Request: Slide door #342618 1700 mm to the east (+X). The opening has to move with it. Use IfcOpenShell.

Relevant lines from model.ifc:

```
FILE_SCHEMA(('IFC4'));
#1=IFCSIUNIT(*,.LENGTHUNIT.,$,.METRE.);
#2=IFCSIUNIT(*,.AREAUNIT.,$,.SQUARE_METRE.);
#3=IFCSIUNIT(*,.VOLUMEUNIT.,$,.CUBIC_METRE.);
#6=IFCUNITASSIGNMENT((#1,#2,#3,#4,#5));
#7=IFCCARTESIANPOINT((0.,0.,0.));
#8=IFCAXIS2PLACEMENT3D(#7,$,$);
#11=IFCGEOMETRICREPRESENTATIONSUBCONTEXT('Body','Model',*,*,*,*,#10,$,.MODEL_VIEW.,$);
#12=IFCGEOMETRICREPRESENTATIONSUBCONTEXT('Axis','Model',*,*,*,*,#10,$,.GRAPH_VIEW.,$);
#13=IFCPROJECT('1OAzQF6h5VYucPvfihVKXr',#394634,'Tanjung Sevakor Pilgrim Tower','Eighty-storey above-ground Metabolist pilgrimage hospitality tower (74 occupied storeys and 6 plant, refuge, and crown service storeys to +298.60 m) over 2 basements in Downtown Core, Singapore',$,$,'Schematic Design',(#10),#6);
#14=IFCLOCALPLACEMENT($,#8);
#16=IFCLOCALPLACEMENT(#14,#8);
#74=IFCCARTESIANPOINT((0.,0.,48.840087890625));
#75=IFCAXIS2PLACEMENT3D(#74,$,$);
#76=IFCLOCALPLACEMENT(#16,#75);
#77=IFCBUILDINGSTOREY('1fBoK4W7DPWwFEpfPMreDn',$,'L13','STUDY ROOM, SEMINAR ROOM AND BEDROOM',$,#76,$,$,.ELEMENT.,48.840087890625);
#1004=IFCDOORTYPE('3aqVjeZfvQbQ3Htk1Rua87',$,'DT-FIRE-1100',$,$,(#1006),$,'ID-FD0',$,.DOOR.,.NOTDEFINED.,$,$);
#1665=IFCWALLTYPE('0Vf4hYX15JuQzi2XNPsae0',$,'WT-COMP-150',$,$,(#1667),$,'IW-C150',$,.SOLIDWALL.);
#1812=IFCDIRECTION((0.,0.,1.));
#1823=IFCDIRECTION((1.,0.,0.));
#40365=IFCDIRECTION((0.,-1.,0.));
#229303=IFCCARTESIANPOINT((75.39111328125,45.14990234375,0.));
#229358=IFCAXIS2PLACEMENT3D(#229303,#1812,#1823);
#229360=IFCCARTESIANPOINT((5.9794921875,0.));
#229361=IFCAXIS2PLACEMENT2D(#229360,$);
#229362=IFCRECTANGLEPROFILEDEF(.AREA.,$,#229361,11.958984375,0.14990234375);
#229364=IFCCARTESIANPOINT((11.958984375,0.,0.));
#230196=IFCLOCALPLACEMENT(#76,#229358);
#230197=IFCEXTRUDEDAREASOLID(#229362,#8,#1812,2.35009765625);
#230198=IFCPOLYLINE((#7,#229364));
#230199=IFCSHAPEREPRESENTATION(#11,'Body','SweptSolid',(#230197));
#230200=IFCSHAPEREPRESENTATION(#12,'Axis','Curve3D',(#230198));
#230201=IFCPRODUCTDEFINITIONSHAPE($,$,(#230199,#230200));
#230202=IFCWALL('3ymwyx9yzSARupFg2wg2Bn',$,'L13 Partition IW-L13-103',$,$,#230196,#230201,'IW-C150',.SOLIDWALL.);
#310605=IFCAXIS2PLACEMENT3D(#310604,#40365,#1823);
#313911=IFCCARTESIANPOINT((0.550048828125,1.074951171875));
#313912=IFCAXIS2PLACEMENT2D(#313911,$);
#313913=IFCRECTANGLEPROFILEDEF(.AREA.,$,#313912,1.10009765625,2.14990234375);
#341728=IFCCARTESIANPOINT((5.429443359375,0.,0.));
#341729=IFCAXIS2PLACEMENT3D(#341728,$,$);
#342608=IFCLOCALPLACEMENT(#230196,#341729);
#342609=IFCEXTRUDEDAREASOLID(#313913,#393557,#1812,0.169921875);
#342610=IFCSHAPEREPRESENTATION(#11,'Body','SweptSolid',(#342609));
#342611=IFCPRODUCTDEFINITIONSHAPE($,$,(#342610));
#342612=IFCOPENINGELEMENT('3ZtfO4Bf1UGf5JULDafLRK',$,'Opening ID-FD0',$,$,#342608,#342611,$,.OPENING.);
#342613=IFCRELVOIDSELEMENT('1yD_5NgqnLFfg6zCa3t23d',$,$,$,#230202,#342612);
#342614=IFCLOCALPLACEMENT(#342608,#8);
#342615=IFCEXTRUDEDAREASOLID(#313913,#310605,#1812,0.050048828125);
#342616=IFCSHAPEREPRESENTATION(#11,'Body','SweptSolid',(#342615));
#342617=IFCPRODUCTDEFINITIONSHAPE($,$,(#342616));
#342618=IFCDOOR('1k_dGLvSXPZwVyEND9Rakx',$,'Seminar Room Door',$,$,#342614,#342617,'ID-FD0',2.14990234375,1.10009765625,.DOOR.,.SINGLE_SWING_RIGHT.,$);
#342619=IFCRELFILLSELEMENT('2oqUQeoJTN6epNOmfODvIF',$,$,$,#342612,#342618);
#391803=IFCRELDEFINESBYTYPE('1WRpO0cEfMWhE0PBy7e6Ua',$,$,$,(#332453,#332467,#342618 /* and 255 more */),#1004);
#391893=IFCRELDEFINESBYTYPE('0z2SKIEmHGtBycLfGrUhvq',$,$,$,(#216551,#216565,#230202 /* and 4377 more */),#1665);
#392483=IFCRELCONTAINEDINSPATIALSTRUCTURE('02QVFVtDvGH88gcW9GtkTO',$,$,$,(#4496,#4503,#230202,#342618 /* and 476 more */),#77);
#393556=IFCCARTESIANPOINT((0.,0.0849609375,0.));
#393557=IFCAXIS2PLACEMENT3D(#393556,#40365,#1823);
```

```python
import ifcopenshell
import ifcopenshell.api.geometry
import ifcopenshell.util.placement

model = ifcopenshell.open("model.ifc")

door = model.by_guid("1k_dGLvSXPZwVyEND9Rakx")
opening = door.FillsVoids[0].RelatingOpeningElement
wall = opening.VoidsElements[0].RelatingBuildingElement

wall_matrix = ifcopenshell.util.placement.get_local_placement(wall.ObjectPlacement)
shift = wall_matrix[:3, 0] * 1.7
before = ifcopenshell.util.placement.get_local_placement(door.ObjectPlacement)[:3, 3].copy()

# The door is placed relative to its opening, so it follows when the opening moves.
matrix = ifcopenshell.util.placement.get_local_placement(opening.ObjectPlacement)
matrix[:3, 3] += shift
ifcopenshell.api.geometry.edit_object_placement(
    model, product=opening, matrix=matrix, is_si=False, should_transform_children=True
)

after = ifcopenshell.util.placement.get_local_placement(door.ObjectPlacement)[:3, 3]
print("door moved by", (after - before).round(3) + 0.0)

model.write("model_edited.ifc")
```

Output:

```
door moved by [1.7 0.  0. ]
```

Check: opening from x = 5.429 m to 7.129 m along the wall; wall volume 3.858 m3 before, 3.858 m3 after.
